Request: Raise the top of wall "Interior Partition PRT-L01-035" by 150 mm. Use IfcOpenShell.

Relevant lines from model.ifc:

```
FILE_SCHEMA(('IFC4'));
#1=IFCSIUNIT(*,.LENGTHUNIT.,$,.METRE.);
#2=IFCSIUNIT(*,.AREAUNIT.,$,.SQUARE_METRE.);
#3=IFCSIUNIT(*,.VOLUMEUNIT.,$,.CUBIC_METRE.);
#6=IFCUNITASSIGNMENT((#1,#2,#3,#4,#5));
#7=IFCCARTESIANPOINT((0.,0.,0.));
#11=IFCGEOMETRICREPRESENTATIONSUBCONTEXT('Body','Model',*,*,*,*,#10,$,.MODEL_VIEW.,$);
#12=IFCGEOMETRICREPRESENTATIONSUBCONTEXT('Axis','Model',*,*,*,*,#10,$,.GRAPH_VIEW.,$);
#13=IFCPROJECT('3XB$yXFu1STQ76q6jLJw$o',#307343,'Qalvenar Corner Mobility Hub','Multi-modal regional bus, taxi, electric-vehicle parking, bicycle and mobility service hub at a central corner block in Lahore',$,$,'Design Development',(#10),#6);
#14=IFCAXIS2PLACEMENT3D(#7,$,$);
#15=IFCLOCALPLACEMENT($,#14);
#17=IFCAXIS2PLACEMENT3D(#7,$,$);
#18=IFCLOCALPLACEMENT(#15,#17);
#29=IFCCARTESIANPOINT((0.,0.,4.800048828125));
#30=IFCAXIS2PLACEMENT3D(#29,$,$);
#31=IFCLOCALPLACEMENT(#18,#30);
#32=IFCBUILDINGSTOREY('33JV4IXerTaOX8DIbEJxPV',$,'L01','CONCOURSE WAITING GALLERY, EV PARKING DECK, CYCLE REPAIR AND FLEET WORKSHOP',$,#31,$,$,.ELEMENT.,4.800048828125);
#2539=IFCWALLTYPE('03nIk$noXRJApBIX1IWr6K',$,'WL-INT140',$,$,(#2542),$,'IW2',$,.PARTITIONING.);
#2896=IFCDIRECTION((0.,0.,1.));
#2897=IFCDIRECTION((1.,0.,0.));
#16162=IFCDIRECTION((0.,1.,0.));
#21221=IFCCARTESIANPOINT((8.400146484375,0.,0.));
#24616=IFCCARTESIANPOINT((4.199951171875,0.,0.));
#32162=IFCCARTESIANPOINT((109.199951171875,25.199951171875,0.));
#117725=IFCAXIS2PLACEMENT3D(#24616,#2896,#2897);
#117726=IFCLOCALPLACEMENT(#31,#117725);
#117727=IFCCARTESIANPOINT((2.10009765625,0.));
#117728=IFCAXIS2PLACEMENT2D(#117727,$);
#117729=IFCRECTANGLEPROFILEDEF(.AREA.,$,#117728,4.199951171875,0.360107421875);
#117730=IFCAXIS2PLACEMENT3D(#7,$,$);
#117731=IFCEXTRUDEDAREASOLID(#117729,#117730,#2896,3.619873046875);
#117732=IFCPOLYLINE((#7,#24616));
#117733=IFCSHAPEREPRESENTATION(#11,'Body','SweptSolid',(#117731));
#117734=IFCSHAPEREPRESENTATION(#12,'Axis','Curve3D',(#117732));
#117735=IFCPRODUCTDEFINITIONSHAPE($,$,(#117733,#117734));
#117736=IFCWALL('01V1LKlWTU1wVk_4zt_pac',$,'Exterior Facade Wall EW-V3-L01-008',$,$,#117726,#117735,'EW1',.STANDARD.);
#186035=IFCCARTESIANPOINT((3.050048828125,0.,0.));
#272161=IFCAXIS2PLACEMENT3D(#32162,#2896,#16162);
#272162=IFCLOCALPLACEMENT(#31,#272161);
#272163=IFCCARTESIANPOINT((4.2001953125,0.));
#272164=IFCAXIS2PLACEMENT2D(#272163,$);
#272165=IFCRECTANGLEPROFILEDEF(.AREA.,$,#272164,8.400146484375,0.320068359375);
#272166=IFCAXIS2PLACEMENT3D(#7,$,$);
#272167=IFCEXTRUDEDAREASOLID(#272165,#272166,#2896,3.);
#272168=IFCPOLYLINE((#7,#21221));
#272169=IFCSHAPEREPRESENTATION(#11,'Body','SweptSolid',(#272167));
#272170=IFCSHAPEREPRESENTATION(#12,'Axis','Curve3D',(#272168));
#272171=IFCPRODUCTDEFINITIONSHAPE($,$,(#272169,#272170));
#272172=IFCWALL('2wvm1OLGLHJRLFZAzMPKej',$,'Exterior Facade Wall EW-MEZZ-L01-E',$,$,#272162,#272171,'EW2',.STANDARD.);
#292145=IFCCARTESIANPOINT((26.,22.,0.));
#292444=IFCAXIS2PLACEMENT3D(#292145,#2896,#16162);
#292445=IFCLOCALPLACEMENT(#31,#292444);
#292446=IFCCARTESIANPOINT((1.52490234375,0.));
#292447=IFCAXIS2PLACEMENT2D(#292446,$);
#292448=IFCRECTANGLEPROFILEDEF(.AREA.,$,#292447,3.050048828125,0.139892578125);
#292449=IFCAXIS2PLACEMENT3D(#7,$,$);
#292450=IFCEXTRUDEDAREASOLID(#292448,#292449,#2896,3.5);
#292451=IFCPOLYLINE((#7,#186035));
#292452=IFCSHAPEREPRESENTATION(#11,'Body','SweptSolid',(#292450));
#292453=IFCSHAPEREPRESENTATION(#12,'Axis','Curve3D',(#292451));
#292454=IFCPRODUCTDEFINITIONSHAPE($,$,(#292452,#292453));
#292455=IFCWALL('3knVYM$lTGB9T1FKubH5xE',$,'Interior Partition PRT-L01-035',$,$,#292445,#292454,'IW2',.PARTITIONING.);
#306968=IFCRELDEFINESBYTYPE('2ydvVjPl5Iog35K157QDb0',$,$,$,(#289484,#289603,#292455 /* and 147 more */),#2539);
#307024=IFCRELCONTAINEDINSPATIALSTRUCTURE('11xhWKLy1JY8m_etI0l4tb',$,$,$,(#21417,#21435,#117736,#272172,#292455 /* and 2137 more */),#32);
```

```python
import ifcopenshell
import ifcopenshell.geom
import ifcopenshell.util.representation
import ifcopenshell.util.shape
import ifcopenshell.util.unit

model = ifcopenshell.open("model.ifc")
unit_scale = ifcopenshell.util.unit.calculate_unit_scale(model)
settings = ifcopenshell.geom.settings()


def volume(element):
    """Net volume in cubic metres, openings subtracted."""
    shape = ifcopenshell.geom.create_shape(settings, element)
    return ifcopenshell.util.shape.get_volume(shape.geometry)


wall = model.by_id(292455)
before = volume(wall)

body = ifcopenshell.util.representation.get_representation(wall, "Model", "Body")
solid = body.Items[0]
old_height = solid.Depth
solid.Depth += 0.15 / unit_scale
after = volume(wall)

print(f"height {old_height:g} -> {solid.Depth:g}, volume {before:.3f} -> {after:.3f} m3")

model.write("model_edited.ifc")
```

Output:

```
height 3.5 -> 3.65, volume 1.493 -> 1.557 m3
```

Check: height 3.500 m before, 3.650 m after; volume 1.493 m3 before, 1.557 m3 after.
